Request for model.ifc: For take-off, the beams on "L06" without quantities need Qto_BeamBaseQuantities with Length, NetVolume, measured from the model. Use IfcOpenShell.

First a look at what the model holds.

```python
import ifcopenshell
import ifcopenshell.util.element
import ifcopenshell.util.unit

model = ifcopenshell.open("model.ifc")
print(model.schema)
for unit_type in ("LENGTHUNIT", "AREAUNIT", "VOLUMEUNIT"):
    print(unit_type, ifcopenshell.util.unit.calculate_unit_scale(model, unit_type))
storey = next(s for s in model.by_type("IfcBuildingStorey") if s.Name == "L06")
beams = [e for e in ifcopenshell.util.element.get_decomposition(storey) if e.is_a("IfcBeam")]
for e in sorted(beams, key=lambda e: e.id()):
    print(e.id(), e.is_a(), e.Name, list(ifcopenshell.util.element.get_psets(e, qtos_only=True)), sep=" | ")
```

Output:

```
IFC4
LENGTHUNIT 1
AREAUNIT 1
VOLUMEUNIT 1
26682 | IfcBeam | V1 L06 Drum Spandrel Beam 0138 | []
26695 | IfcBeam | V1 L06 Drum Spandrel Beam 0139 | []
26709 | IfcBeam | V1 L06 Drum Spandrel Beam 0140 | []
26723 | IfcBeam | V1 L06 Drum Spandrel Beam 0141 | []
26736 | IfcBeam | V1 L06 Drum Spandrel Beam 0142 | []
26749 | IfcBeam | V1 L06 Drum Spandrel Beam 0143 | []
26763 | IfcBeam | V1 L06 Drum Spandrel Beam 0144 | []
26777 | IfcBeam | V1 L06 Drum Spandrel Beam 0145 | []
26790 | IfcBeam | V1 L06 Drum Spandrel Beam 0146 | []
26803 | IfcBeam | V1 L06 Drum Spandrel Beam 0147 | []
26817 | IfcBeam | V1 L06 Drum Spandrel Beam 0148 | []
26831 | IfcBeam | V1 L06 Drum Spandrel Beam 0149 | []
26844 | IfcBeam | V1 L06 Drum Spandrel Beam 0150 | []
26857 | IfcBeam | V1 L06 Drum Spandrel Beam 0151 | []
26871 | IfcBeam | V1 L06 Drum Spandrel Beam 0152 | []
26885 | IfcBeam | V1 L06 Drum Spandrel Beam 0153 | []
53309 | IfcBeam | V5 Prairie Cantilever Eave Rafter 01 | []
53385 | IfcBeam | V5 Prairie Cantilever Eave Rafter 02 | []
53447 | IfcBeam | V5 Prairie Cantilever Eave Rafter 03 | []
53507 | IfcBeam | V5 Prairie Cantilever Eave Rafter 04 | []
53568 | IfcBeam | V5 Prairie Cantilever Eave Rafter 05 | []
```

```python
import ifcopenshell
import ifcopenshell.api.pset
import ifcopenshell.geom
import ifcopenshell.util.element
import ifcopenshell.util.shape
import ifcopenshell.util.unit

model = ifcopenshell.open("model.ifc")
unit_scale = ifcopenshell.util.unit.calculate_unit_scale(model)
volume_scale = ifcopenshell.util.unit.calculate_unit_scale(model, "VOLUMEUNIT")
settings = ifcopenshell.geom.settings()

storey = next(s for s in model.by_type("IfcBuildingStorey") if s.Name == "L06")
beams = [e for e in ifcopenshell.util.element.get_decomposition(storey) if e.is_a("IfcBeam")]

for e in sorted(beams, key=lambda e: e.id()):
    if ifcopenshell.util.element.get_psets(e, qtos_only=True, should_inherit=False):
        continue
    # Geometry comes back in metres, in the element's own axes.
    shape = ifcopenshell.geom.create_shape(settings, e)
    values = {
        "Length": ifcopenshell.util.shape.get_max_xyz(shape.geometry) / unit_scale,
        "NetVolume": ifcopenshell.util.shape.get_volume(shape.geometry) / volume_scale,
    }
    qto = ifcopenshell.api.pset.add_qto(model, product=e, name="Qto_BeamBaseQuantities")
    ifcopenshell.api.pset.edit_qto(model, qto=qto, properties=values)
    print(e.id(), {k: round(v, 3) for k, v in values.items()})

model.write("model_updated.ifc")
```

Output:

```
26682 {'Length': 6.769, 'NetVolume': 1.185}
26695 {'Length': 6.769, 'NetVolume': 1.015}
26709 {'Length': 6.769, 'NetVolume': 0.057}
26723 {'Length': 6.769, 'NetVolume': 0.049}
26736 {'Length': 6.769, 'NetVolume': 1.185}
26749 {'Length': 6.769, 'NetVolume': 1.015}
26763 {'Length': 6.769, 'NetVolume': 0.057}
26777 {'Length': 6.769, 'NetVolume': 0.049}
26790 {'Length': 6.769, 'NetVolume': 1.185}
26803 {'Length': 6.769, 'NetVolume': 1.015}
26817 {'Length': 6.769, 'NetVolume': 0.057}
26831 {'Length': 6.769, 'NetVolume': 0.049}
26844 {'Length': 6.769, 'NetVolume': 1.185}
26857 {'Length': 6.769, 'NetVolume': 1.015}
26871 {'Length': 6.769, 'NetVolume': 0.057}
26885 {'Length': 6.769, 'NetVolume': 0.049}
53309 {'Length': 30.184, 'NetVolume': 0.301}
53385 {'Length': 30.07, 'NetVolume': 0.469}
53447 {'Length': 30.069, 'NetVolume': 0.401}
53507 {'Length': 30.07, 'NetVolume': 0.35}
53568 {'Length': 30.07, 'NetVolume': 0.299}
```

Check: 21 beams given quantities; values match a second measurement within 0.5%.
